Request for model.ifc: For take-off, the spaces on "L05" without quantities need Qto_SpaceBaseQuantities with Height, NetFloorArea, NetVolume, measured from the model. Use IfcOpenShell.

First a look at what the model holds.

```python
import ifcopenshell
import ifcopenshell.util.element
import ifcopenshell.util.unit

model = ifcopenshell.open("model.ifc")
print(model.schema)
for unit_type in ("LENGTHUNIT", "AREAUNIT", "VOLUMEUNIT"):
    print(unit_type, ifcopenshell.util.unit.calculate_unit_scale(model, unit_type))
storey = next(s for s in model.by_type("IfcBuildingStorey") if s.Name == "L05")
spaces = [e for e in ifcopenshell.util.element.get_decomposition(storey) if e.is_a("IfcSpace")]
for e in sorted(spaces, key=lambda e: e.id()):
    print(e.id(), e.is_a(), e.Name, list(ifcopenshell.util.element.get_psets(e, qtos_only=True)), sep=" | ")
```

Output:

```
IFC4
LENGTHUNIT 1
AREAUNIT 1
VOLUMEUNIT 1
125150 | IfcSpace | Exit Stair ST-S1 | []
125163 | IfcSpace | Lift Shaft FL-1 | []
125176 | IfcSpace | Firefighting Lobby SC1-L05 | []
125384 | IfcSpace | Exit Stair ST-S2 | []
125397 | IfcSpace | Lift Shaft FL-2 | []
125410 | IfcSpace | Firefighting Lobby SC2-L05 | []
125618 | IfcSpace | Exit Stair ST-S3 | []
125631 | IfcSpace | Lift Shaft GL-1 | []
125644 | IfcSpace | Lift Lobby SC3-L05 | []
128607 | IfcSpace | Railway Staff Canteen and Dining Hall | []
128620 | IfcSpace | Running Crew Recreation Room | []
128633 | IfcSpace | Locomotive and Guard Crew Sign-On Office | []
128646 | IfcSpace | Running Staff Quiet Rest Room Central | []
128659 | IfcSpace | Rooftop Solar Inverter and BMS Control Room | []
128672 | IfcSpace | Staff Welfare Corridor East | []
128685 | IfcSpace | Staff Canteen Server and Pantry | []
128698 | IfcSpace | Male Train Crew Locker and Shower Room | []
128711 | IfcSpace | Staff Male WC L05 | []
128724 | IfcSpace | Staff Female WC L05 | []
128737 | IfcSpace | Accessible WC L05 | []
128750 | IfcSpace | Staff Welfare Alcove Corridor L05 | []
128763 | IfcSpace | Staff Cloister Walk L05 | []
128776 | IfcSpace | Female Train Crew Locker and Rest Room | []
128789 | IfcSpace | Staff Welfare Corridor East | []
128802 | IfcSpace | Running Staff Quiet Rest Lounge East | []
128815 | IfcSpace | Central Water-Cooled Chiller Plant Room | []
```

```python
import ifcopenshell
import ifcopenshell.api.pset
import ifcopenshell.geom
import ifcopenshell.util.element
import ifcopenshell.util.shape
import ifcopenshell.util.unit

model = ifcopenshell.open("model.ifc")
unit_scale = ifcopenshell.util.unit.calculate_unit_scale(model)
area_scale = ifcopenshell.util.unit.calculate_unit_scale(model, "AREAUNIT")
volume_scale = ifcopenshell.util.unit.calculate_unit_scale(model, "VOLUMEUNIT")
settings = ifcopenshell.geom.settings()

storey = next(s for s in model.by_type("IfcBuildingStorey") if s.Name == "L05")
spaces = [e for e in ifcopenshell.util.element.get_decomposition(storey) if e.is_a("IfcSpace")]

for e in sorted(spaces, key=lambda e: e.id()):
    if ifcopenshell.util.element.get_psets(e, qtos_only=True, should_inherit=False):
        continue
    # Geometry comes back in metres, in the element's own axes.
    shape = ifcopenshell.geom.create_shape(settings, e)
    values = {
        "Height": ifcopenshell.util.shape.get_z(shape.geometry) / unit_scale,
        "NetFloorArea": ifcopenshell.util.shape.get_footprint_area(shape.geometry) / area_scale,
        "NetVolume": ifcopenshell.util.shape.get_volume(shape.geometry) / volume_scale,
    }
    qto = ifcopenshell.api.pset.add_qto(model, product=e, name="Qto_SpaceBaseQuantities")
    ifcopenshell.api.pset.edit_qto(model, qto=qto, properties=values)
    print(e.id(), {k: round(v, 3) for k, v in values.items()})

model.write("model_v2.ifc")
```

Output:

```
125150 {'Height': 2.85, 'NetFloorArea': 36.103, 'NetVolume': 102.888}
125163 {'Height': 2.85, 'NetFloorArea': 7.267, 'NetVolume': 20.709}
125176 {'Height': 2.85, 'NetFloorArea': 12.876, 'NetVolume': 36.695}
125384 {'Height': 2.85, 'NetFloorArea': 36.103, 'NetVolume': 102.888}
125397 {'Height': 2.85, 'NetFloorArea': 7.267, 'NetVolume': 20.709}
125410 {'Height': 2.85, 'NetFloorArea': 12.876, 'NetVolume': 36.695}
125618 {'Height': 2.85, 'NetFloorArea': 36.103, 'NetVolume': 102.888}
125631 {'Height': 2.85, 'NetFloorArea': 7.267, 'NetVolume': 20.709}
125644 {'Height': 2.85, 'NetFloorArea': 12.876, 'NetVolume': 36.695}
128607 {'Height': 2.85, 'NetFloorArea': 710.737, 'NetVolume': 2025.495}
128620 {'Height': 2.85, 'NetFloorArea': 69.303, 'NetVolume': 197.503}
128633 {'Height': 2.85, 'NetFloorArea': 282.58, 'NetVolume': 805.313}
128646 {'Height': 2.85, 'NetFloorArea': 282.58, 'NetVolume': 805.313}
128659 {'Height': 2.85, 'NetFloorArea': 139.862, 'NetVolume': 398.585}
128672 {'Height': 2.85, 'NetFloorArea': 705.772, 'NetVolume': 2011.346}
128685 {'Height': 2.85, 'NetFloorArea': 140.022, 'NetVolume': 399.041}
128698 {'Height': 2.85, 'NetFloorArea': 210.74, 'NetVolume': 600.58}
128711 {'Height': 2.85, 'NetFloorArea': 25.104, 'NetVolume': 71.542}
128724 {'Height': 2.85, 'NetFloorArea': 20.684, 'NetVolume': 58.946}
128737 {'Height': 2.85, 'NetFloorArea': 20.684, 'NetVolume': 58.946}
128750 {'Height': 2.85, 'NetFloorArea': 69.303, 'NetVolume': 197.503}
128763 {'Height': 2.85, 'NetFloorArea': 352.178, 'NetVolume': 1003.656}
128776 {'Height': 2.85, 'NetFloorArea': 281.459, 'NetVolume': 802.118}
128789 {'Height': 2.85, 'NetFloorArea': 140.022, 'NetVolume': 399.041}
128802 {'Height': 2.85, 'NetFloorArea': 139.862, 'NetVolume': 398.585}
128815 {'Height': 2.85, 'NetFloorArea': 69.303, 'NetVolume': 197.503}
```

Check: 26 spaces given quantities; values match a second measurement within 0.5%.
